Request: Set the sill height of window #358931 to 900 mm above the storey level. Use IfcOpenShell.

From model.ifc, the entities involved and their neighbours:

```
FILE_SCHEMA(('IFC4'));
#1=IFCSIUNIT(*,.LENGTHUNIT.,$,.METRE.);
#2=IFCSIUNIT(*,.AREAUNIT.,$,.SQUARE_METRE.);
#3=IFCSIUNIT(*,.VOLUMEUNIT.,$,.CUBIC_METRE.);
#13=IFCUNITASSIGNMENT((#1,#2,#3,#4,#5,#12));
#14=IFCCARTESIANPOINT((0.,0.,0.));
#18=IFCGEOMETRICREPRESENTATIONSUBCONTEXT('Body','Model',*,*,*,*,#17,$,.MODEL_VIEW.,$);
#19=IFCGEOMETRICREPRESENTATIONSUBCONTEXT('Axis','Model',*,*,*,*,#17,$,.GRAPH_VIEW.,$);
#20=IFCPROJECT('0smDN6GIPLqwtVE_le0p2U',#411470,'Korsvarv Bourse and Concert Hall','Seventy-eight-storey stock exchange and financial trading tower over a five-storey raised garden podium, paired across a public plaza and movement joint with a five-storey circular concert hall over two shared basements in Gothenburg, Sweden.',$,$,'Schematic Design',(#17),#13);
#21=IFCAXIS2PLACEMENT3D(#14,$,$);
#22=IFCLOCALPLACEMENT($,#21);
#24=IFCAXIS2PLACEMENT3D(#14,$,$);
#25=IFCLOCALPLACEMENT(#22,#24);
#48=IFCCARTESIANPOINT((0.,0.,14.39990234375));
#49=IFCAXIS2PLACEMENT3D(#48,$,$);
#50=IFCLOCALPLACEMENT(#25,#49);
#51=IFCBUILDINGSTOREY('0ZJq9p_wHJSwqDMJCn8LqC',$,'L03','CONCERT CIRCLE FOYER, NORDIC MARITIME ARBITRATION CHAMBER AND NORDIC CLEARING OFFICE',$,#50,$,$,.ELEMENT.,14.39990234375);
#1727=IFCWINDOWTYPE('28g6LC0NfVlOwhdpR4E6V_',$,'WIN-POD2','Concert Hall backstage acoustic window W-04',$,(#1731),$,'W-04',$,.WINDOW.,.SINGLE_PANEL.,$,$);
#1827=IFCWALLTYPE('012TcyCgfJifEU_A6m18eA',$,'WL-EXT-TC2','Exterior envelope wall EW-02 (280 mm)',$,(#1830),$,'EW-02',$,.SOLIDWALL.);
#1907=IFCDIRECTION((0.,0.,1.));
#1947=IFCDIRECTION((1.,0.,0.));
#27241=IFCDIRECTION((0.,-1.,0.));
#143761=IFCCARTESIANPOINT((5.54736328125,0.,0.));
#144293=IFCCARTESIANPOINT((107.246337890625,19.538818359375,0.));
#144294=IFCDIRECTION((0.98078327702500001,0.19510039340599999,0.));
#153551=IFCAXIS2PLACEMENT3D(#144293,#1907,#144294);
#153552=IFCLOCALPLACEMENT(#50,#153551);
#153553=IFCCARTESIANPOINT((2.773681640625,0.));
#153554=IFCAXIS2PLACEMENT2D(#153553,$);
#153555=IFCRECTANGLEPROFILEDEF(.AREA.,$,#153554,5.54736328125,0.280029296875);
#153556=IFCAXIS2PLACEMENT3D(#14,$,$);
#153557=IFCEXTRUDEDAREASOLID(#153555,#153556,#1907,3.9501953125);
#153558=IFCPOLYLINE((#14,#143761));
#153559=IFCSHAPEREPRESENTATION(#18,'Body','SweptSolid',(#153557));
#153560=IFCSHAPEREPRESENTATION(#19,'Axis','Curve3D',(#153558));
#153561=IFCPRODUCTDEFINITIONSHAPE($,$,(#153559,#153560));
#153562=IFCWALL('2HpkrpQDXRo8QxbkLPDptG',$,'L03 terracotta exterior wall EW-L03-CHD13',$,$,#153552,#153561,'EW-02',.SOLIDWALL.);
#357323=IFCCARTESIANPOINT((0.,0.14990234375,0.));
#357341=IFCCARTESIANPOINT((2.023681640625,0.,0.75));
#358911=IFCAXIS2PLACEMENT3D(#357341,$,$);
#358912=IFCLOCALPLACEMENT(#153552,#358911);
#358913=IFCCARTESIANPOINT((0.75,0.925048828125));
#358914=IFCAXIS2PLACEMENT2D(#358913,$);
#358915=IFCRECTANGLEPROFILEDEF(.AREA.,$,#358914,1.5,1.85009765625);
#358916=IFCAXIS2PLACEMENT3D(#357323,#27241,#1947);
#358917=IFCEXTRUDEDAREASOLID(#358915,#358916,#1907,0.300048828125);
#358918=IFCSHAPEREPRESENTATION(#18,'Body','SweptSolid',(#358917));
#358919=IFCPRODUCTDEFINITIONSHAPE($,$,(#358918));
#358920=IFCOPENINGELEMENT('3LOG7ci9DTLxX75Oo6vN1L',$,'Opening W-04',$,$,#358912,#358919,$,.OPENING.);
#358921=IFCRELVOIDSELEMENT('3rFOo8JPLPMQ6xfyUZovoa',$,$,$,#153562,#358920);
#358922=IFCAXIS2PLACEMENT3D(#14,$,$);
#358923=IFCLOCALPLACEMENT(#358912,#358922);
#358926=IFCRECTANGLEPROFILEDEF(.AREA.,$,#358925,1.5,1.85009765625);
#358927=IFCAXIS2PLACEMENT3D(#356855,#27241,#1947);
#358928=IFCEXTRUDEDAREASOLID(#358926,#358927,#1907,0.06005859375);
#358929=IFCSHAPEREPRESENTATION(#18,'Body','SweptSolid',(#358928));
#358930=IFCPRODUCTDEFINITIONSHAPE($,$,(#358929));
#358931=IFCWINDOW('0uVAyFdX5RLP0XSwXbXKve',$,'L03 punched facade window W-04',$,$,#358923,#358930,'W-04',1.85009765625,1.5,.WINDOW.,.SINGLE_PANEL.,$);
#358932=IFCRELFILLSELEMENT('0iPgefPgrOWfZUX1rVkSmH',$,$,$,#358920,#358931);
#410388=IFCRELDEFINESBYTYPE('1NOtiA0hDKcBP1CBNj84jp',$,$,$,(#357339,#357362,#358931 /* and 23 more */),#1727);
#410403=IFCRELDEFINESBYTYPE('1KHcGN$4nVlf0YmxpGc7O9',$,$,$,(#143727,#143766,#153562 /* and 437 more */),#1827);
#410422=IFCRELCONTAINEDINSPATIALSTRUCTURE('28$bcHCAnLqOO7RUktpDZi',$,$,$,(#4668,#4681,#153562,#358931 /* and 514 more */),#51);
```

```python
import numpy as np
import ifcopenshell
import ifcopenshell.api.geometry
import ifcopenshell.geom
import ifcopenshell.util.element
import ifcopenshell.util.placement
import ifcopenshell.util.shape
import ifcopenshell.util.unit

model = ifcopenshell.open("model.ifc")
unit_scale = ifcopenshell.util.unit.calculate_unit_scale(model)

window = model.by_guid("0uVAyFdX5RLP0XSwXbXKve")
opening = window.FillsVoids[0].RelatingOpeningElement
storey = ifcopenshell.util.element.get_container(window, ifc_class="IfcBuildingStorey")
level = ifcopenshell.util.placement.get_local_placement(storey.ObjectPlacement)[2, 3]

# The opening's origin need not be at the sill, so measure its lowest point.
shape = ifcopenshell.geom.create_shape(ifcopenshell.geom.settings(), opening)
bottom = ifcopenshell.util.shape.get_shape_bottom_elevation(shape, shape.geometry) / unit_scale
dz = level + 0.9 / unit_scale - bottom

shift = np.array([0.0, 0.0, dz])
# The window is placed relative to its opening, so it follows when the opening moves.
matrix = ifcopenshell.util.placement.get_local_placement(opening.ObjectPlacement)
matrix[:3, 3] += shift
ifcopenshell.api.geometry.edit_object_placement(
    model, product=opening, matrix=matrix, is_si=False, should_transform_children=True
)

print(f"moved by {dz * unit_scale:+.3f} m")

model.write("model_updated.ifc")
```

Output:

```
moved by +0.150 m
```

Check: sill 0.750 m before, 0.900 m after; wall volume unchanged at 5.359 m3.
